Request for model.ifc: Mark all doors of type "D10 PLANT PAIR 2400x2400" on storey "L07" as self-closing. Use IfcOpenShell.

First a look at what the model holds.

```python
import ifcopenshell
import ifcopenshell.util.element

model = ifcopenshell.open("model.ifc")
print(model.schema)
storey = next(s for s in model.by_type("IfcBuildingStorey") if s.Name == "L07")
doors = [e for e in ifcopenshell.util.element.get_decomposition(storey) if e.is_a("IfcDoor")]
seen = {}
for e in doors:
    element_type = ifcopenshell.util.element.get_type(e)
    key = (element_type.Name if element_type != e and element_type else None, ifcopenshell.util.element.get_pset(e, "Pset_DoorCommon", "SelfClosing"))
    seen[key] = seen.get(key, 0) + 1
for (name, value), count in sorted(seen.items(), key=str):
    print(count, "x", name, "|", value)
```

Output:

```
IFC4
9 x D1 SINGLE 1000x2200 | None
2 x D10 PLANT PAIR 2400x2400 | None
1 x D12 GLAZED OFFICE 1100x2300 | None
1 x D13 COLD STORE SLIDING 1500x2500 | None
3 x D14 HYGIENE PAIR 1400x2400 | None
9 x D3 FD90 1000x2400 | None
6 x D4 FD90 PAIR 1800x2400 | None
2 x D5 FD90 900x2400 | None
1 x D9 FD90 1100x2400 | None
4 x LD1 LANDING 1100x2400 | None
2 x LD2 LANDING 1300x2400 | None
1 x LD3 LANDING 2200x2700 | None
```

```python
import ifcopenshell
import ifcopenshell.api.pset
import ifcopenshell.util.element

model = ifcopenshell.open("model.ifc")

storey = next(s for s in model.by_type("IfcBuildingStorey") if s.Name == "L07")
doors = [e for e in ifcopenshell.util.element.get_decomposition(storey) if e.is_a("IfcDoor")]

count = 0
for e in doors:
    element_type = ifcopenshell.util.element.get_type(e)
    if element_type in (None, e) or element_type.Name != "D10 PLANT PAIR 2400x2400":
        continue
    # add_pset returns the element's existing set when there is one.
    pset = ifcopenshell.api.pset.add_pset(model, product=e, name="Pset_DoorCommon")
    ifcopenshell.api.pset.edit_pset(model, pset=pset, properties={"SelfClosing": True})
    count += 1

print(count, "doors updated")

model.write("model-out.ifc")
```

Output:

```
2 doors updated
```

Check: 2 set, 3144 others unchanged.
